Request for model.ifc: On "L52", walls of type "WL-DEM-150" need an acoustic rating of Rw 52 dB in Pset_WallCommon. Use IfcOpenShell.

First a look at what the model holds.

```python
import ifcopenshell
import ifcopenshell.util.element

model = ifcopenshell.open("model.ifc")
print(model.schema)
storey = next(s for s in model.by_type("IfcBuildingStorey") if s.Name == "L52")
walls = [e for e in ifcopenshell.util.element.get_decomposition(storey) if e.is_a("IfcWall")]
seen = {}
for e in walls:
    element_type = ifcopenshell.util.element.get_type(e)
    key = (element_type.Name if element_type != e and element_type else None, ifcopenshell.util.element.get_pset(e, "Pset_WallCommon", "AcousticRating"))
    seen[key] = seen.get(key, 0) + 1
for (name, value), count in sorted(seen.items(), key=str):
    print(count, "x", name, "|", value)
```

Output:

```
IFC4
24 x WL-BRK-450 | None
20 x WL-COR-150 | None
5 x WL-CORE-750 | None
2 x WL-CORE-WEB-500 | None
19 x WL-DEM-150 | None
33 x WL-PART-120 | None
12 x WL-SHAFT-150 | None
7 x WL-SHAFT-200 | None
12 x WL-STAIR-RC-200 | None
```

```python
import ifcopenshell
import ifcopenshell.api.pset
import ifcopenshell.util.element

model = ifcopenshell.open("model.ifc")

storey = next(s for s in model.by_type("IfcBuildingStorey") if s.Name == "L52")
walls = [e for e in ifcopenshell.util.element.get_decomposition(storey) if e.is_a("IfcWall")]

count = 0
for e in walls:
    element_type = ifcopenshell.util.element.get_type(e)
    if element_type in (None, e) or element_type.Name != "WL-DEM-150":
        continue
    # add_pset returns the element's existing set when there is one.
    pset = ifcopenshell.api.pset.add_pset(model, product=e, name="Pset_WallCommon")
    ifcopenshell.api.pset.edit_pset(model, pset=pset, properties={"AcousticRating": "Rw 52 dB"})
    count += 1

print(count, "walls updated")

model.write("model_updated.ifc")
```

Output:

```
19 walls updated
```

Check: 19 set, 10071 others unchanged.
